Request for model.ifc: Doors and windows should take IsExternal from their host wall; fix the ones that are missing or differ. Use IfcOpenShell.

First a look at what the model holds.

```python
import ifcopenshell
import ifcopenshell.util.element

model = ifcopenshell.open("model.ifc")
print(model.schema)
seen = {}
for e in model.by_type("IfcDoor") + model.by_type("IfcWindow"):
    if not e.FillsVoids:
        continue
    host = e.FillsVoids[0].RelatingOpeningElement.VoidsElements[0].RelatingBuildingElement
    own = ifcopenshell.util.element.get_pset(e, f"Pset_{e.is_a()[3:].removesuffix('StandardCase')}Common", "IsExternal")
    wall = ifcopenshell.util.element.get_pset(host, "Pset_WallCommon", "IsExternal")
    seen[e.is_a(), own, wall] = seen.get((e.is_a(), own, wall), 0) + 1
for (cls, own, wall), count in sorted(seen.items(), key=str):
    print(count, cls, "IsExternal:", own, "| host wall:", wall)
```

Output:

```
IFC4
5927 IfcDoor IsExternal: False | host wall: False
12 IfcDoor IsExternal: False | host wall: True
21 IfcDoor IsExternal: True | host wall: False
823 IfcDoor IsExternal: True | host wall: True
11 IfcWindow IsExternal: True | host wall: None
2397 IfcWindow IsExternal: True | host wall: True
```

```python
import ifcopenshell
import ifcopenshell.api.pset
import ifcopenshell.util.element

model = ifcopenshell.open("model.ifc")

count = 0
for ifc_class, pset_name in (("IfcDoor", "Pset_DoorCommon"), ("IfcWindow", "Pset_WindowCommon")):
    for e in model.by_type(ifc_class):
        if not e.FillsVoids:
            continue
        host = e.FillsVoids[0].RelatingOpeningElement.VoidsElements[0].RelatingBuildingElement
        external = ifcopenshell.util.element.get_pset(host, "Pset_WallCommon", "IsExternal")
        if external is None or ifcopenshell.util.element.get_pset(e, pset_name, "IsExternal") == external:
            continue
        found = ifcopenshell.util.element.get_pset(e, pset_name, should_inherit=False)
        if found:
            pset = model.by_id(found["id"])
            if len(ifcopenshell.util.element.get_elements_by_pset(pset)) > 1:
                pset = ifcopenshell.api.pset.unshare_pset(model, products=[e], pset=pset)[0]
        else:
            pset = ifcopenshell.api.pset.add_pset(model, product=e, name=pset_name)
        ifcopenshell.api.pset.edit_pset(model, pset=pset, properties={"IsExternal": external})
        count += 1

print(count, "updated")

model.write("model-out.ifc")
```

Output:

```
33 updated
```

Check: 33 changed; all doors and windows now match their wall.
